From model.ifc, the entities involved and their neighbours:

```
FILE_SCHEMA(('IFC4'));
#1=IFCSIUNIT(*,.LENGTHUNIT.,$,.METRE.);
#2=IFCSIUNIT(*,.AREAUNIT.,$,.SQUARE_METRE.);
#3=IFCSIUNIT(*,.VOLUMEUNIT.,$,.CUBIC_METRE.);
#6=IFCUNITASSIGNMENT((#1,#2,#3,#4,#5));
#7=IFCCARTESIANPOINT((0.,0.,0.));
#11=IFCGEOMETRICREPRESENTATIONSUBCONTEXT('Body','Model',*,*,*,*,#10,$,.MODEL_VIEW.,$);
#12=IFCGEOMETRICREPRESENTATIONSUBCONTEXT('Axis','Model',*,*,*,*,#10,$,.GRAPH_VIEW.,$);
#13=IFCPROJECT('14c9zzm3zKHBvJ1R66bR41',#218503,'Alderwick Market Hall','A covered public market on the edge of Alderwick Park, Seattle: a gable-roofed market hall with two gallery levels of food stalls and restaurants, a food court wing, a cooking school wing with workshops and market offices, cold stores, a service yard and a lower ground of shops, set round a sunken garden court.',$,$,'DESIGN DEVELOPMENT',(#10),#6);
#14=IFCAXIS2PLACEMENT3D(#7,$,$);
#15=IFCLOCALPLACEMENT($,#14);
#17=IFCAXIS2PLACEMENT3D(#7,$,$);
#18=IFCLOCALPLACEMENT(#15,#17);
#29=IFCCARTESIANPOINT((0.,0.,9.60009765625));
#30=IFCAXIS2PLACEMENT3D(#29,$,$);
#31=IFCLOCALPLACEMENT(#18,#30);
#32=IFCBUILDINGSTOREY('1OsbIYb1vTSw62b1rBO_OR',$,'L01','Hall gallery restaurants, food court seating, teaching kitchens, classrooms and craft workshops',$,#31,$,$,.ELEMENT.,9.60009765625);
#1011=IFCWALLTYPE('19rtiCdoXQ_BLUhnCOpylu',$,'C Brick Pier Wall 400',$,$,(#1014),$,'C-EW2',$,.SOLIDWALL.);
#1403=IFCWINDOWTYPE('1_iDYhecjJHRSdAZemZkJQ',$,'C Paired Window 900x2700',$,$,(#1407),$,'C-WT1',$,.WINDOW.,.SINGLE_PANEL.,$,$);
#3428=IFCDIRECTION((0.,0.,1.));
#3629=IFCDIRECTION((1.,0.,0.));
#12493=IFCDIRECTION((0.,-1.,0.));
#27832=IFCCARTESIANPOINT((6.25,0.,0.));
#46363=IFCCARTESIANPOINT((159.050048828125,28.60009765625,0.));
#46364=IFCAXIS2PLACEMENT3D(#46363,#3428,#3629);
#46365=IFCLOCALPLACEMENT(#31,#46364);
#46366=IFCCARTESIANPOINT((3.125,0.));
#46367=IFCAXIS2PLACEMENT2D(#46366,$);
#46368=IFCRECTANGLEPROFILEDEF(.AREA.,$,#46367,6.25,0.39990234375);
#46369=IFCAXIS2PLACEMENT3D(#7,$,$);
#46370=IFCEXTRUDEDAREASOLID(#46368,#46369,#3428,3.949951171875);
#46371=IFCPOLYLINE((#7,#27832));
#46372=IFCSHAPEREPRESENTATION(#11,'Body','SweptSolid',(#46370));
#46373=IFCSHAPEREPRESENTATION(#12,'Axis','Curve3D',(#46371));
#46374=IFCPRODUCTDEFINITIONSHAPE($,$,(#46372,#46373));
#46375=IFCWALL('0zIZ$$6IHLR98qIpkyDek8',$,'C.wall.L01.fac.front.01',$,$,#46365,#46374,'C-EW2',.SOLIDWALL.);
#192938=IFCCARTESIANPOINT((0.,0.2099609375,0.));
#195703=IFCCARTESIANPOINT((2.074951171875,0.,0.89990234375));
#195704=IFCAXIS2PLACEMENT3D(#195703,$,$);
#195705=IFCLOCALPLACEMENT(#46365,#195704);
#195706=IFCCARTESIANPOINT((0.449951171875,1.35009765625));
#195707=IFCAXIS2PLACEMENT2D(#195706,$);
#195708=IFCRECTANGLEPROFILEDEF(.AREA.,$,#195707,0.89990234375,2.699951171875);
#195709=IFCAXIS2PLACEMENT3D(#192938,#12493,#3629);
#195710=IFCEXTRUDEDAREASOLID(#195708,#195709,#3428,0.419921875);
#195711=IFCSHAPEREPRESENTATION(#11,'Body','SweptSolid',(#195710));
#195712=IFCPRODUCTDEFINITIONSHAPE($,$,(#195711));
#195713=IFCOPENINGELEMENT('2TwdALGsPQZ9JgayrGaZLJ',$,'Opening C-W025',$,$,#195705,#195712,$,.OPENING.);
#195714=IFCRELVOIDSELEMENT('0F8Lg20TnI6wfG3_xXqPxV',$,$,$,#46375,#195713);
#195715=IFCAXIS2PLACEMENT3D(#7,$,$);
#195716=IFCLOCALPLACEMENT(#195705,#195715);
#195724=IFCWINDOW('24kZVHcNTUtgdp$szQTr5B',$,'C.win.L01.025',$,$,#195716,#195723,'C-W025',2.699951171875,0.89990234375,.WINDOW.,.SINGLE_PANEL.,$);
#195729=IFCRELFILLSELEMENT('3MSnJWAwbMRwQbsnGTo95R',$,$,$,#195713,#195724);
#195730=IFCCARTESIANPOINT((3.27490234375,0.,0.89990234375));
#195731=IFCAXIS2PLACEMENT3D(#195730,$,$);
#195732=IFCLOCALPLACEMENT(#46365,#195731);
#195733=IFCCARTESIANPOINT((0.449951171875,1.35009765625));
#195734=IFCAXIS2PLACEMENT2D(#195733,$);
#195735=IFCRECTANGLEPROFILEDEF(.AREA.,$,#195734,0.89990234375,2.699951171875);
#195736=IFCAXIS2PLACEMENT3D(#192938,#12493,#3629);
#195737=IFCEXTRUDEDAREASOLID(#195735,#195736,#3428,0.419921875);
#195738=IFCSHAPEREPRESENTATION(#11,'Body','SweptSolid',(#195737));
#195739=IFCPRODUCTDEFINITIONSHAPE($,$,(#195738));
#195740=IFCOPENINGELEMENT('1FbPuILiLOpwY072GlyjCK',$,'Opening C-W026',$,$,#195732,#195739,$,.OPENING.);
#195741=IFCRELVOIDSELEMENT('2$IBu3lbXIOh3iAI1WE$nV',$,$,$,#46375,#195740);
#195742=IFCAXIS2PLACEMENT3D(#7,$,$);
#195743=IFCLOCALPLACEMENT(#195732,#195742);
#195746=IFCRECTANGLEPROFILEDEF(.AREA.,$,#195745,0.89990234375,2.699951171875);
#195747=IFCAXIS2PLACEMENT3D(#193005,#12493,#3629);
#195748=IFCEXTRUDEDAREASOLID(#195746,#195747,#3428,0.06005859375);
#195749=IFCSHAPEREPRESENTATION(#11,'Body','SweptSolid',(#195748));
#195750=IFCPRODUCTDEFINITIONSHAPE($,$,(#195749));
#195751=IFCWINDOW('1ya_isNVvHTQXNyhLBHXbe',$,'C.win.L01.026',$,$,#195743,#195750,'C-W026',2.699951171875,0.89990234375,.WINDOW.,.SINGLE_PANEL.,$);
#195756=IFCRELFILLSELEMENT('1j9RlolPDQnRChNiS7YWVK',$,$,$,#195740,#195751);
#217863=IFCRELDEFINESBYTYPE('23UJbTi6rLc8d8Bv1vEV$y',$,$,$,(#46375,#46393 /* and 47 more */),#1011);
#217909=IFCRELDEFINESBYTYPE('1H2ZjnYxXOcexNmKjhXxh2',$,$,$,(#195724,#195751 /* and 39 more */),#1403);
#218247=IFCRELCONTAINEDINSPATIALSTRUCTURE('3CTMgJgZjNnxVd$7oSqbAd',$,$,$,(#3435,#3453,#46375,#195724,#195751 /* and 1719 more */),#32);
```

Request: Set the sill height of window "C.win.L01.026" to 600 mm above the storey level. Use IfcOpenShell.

```python
import numpy as np
import ifcopenshell
import ifcopenshell.api.geometry
import ifcopenshell.geom
import ifcopenshell.util.element
import ifcopenshell.util.placement
import ifcopenshell.util.shape
import ifcopenshell.util.unit

model = ifcopenshell.open("model.ifc")
unit_scale = ifcopenshell.util.unit.calculate_unit_scale(model)

window = model.by_guid("1ya_isNVvHTQXNyhLBHXbe")
opening = window.FillsVoids[0].RelatingOpeningElement
storey = ifcopenshell.util.element.get_container(window, ifc_class="IfcBuildingStorey")
level = ifcopenshell.util.placement.get_local_placement(storey.ObjectPlacement)[2, 3]

# The opening's origin need not be at the sill, so measure its lowest point.
shape = ifcopenshell.geom.create_shape(ifcopenshell.geom.settings(), opening)
bottom = ifcopenshell.util.shape.get_shape_bottom_elevation(shape, shape.geometry) / unit_scale
dz = level + 0.6 / unit_scale - bottom

shift = np.array([0.0, 0.0, dz])
# The window is placed relative to its opening, so it follows when the opening moves.
matrix = ifcopenshell.util.placement.get_local_placement(opening.ObjectPlacement)
matrix[:3, 3] += shift
ifcopenshell.api.geometry.edit_object_placement(
    model, product=opening, matrix=matrix, is_si=False, should_transform_children=True
)

print(f"moved by {dz * unit_scale:+.3f} m")

model.write("model-out.ifc")
```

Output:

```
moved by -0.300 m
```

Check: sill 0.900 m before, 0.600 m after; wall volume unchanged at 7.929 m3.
